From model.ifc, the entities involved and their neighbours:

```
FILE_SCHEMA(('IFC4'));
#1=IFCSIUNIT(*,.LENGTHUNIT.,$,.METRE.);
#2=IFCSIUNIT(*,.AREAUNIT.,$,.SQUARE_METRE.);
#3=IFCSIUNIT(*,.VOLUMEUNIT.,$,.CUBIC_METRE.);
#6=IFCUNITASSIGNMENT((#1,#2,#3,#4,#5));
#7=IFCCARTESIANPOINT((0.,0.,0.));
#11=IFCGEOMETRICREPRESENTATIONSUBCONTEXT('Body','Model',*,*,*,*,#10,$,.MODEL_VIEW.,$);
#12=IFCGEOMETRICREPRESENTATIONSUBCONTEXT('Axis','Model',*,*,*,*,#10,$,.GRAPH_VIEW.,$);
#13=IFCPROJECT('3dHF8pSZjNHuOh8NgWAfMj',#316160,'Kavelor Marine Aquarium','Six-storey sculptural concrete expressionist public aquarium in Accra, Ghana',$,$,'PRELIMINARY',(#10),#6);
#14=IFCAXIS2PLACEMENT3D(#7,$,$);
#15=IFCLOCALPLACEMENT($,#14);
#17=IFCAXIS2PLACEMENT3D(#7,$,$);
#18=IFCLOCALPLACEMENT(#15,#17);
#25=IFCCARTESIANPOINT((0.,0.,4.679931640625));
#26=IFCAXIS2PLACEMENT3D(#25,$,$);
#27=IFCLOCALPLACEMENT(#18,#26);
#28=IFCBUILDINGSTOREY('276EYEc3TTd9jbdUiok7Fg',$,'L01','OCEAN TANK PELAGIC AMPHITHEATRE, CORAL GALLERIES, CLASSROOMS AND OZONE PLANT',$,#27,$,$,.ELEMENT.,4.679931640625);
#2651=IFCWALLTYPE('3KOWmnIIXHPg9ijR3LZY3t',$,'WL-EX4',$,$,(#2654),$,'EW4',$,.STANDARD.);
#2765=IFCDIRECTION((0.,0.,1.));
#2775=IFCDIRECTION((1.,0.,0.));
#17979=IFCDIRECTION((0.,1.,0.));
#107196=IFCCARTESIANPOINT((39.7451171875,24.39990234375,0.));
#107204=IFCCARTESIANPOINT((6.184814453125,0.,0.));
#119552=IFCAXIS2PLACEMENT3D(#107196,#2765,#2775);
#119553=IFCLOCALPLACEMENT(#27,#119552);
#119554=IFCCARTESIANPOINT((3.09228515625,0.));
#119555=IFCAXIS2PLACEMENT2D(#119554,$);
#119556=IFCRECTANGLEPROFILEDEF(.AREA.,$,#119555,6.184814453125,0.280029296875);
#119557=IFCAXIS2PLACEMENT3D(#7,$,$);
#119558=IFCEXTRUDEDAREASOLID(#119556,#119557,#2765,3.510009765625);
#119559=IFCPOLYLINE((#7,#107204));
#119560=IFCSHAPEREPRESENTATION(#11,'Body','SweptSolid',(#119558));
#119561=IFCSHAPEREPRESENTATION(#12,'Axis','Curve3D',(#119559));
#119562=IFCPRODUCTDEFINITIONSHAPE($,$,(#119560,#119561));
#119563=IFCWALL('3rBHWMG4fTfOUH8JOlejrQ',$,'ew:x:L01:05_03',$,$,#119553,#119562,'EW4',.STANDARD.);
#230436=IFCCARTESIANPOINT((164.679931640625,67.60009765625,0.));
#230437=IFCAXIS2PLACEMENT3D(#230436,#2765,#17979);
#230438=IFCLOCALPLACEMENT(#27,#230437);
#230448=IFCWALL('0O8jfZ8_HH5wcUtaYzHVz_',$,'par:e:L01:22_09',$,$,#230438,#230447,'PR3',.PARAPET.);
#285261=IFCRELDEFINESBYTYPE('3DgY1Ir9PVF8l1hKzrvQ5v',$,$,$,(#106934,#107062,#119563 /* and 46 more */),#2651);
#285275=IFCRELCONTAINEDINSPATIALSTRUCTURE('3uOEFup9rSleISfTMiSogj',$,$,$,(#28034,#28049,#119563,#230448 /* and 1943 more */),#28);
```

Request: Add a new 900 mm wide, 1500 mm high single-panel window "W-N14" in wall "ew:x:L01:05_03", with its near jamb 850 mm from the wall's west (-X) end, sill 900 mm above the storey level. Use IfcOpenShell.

```python
import numpy as np
import ifcopenshell
import ifcopenshell.api.feature
import ifcopenshell.api.geometry
import ifcopenshell.api.root
import ifcopenshell.api.spatial
import ifcopenshell.geom
import ifcopenshell.util.element
import ifcopenshell.util.placement
import ifcopenshell.util.representation
import ifcopenshell.util.shape
import ifcopenshell.util.unit

model = ifcopenshell.open("model.ifc")
unit_scale = ifcopenshell.util.unit.calculate_unit_scale(model)
settings = ifcopenshell.geom.settings()


def volume(element):
    """Net volume in cubic metres, openings subtracted."""
    shape = ifcopenshell.geom.create_shape(settings, element)
    return ifcopenshell.util.shape.get_volume(shape.geometry)


wall = model.by_id(119563)
storey = ifcopenshell.util.element.get_container(wall, ifc_class="IfcBuildingStorey")
context = ifcopenshell.util.representation.get_context(model, "Model", "Body", "MODEL_VIEW")
before = volume(wall)

width, height, from_end, sill = 0.9, 1.5, 0.85, 0.9  # metres

# The wall runs along its own X axis, and the end named is its -X end.
wall_shape = ifcopenshell.geom.create_shape(settings, wall)
x, y, z = ifcopenshell.util.shape.get_vertices(wall_shape.geometry).T
start = x.min() + from_end
face, thickness = float(y.min()), float(y.max() - y.min())
wall_matrix = ifcopenshell.util.placement.get_local_placement(wall.ObjectPlacement)
level = ifcopenshell.util.placement.get_local_placement(storey.ObjectPlacement)[2, 3]


def in_wall(x, y):
    """Placement at x, y metres in the wall's axes, at sill height."""
    matrix = wall_matrix.copy()
    matrix[:, 3] = wall_matrix @ np.array([x / unit_scale, y / unit_scale, 0.0, 1.0])
    matrix[2, 3] = level + sill / unit_scale
    return matrix


# Opening: a box that overshoots both wall faces by 50 mm.
opening = ifcopenshell.api.root.create_entity(model, ifc_class="IfcOpeningElement", predefined_type="OPENING")
box = ifcopenshell.api.geometry.add_wall_representation(
    model, context=context, length=width, height=height, thickness=thickness + 0.1
)
ifcopenshell.api.geometry.assign_representation(model, product=opening, representation=box)
ifcopenshell.api.geometry.edit_object_placement(model, product=opening, matrix=in_wall(start, face - 0.05), is_si=False)
ifcopenshell.api.feature.add_feature(model, feature=opening, element=wall)

window = ifcopenshell.api.root.create_entity(model, ifc_class="IfcWindow", name="W-N14", predefined_type="WINDOW")
window.OverallWidth, window.OverallHeight = width / unit_scale, height / unit_scale
window.PartitioningType = "SINGLE_PANEL"
body = ifcopenshell.api.geometry.add_window_representation(
    model,
    context=context,
    overall_width=window.OverallWidth,
    overall_height=window.OverallHeight,
    partition_type="SINGLE_PANEL",
)
ifcopenshell.api.geometry.assign_representation(model, product=window, representation=body)
ifcopenshell.api.spatial.assign_container(model, products=[window], relating_structure=storey)
ifcopenshell.api.feature.add_filling(model, opening=opening, element=window)

# Centre the window in the wall's thickness.
ifcopenshell.api.geometry.edit_object_placement(model, product=window, matrix=in_wall(start, face), is_si=False)
window_shape = ifcopenshell.geom.create_shape(settings, window)
depth = ifcopenshell.util.shape.get_vertices(window_shape.geometry)[:, 1]
offset = face + thickness / 2 - (depth.min() + depth.max()) / 2
ifcopenshell.api.geometry.edit_object_placement(model, product=window, matrix=in_wall(start, offset), is_si=False)

after = volume(wall)

print(f"wall volume {before:.3f} -> {after:.3f} m3")

model.write("model_rev.ifc")
```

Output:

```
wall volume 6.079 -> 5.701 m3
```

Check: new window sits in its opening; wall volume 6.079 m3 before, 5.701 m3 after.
